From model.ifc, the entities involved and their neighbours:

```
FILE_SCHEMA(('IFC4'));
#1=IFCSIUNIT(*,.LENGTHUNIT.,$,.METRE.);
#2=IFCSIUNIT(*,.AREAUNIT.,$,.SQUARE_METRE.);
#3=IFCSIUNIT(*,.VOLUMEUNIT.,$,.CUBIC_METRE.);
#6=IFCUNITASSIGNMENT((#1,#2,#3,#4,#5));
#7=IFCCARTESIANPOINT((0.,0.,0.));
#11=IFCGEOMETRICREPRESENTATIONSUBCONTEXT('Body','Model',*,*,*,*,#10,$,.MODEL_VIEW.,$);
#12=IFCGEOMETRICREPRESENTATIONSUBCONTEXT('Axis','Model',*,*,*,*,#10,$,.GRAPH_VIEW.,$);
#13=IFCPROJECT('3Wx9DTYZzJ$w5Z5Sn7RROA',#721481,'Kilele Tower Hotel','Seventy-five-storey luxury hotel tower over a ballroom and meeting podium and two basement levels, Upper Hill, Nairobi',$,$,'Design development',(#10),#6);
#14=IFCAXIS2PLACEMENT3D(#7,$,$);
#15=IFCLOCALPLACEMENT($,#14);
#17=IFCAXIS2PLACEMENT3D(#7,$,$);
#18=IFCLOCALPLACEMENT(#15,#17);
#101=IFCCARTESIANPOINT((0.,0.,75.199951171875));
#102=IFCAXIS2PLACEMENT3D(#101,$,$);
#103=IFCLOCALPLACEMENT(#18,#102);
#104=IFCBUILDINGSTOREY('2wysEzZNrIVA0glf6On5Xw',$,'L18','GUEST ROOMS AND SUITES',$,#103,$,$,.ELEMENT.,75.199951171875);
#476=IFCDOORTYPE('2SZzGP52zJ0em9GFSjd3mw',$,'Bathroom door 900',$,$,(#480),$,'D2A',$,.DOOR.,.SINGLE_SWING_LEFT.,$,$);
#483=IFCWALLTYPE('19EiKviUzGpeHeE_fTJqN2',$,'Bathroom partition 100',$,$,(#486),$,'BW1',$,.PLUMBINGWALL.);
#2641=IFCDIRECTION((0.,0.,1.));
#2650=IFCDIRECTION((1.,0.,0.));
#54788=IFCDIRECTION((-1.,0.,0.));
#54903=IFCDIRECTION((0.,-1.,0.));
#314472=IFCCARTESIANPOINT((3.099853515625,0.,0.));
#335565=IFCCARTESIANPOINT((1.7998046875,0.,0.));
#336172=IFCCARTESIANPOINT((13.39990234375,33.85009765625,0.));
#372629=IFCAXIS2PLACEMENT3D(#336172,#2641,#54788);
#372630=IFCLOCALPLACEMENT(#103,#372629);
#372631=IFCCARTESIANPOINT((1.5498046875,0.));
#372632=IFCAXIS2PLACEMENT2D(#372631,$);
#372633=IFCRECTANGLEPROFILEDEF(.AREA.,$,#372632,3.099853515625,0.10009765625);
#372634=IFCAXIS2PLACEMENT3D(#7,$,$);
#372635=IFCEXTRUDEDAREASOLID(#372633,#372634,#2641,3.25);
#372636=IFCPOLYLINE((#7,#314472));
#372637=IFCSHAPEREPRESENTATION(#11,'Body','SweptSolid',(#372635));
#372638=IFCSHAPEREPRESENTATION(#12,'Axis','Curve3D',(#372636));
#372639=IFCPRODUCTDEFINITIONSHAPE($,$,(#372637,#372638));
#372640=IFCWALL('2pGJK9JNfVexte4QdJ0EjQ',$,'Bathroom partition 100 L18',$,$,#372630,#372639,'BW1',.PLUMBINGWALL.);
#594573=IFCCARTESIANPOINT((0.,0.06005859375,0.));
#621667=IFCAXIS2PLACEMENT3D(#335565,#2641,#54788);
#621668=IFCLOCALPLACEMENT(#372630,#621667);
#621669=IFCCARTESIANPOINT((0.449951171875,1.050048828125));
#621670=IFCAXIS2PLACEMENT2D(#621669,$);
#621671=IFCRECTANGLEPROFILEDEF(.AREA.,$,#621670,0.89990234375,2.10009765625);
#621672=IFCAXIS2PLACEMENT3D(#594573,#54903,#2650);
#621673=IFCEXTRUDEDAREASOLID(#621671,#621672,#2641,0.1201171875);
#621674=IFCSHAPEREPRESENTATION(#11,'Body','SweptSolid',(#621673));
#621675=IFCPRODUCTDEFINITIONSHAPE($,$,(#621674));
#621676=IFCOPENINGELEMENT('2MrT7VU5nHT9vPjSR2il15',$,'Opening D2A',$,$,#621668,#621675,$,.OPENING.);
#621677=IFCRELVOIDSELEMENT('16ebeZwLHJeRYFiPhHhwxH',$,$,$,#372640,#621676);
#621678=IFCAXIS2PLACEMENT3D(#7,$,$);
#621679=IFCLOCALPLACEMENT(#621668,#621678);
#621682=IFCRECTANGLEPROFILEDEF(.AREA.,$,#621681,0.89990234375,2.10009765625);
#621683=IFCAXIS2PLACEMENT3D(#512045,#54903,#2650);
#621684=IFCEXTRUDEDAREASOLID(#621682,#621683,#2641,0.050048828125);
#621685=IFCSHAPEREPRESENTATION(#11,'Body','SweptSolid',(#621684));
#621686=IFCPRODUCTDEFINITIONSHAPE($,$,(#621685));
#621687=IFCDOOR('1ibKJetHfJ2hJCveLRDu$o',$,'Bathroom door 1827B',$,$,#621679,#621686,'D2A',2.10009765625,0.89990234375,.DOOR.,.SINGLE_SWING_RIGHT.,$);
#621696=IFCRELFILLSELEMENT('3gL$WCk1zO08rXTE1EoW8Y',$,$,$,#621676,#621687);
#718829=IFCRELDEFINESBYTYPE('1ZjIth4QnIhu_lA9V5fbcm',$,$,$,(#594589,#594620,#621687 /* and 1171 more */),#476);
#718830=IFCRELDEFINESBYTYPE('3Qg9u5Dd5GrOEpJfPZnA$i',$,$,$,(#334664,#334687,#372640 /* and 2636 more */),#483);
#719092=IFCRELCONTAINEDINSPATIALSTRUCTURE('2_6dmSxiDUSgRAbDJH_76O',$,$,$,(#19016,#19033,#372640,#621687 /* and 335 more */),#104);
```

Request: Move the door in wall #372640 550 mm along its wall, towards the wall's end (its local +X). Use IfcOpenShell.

```python
import ifcopenshell
import ifcopenshell.api.geometry
import ifcopenshell.util.placement

model = ifcopenshell.open("model.ifc")

door = model.by_id(621687)
opening = door.FillsVoids[0].RelatingOpeningElement
wall = opening.VoidsElements[0].RelatingBuildingElement

wall_matrix = ifcopenshell.util.placement.get_local_placement(wall.ObjectPlacement)
shift = wall_matrix[:3, 0] * 0.55
before = ifcopenshell.util.placement.get_local_placement(door.ObjectPlacement)[:3, 3].copy()

# The door is placed relative to its opening, so it follows when the opening moves.
matrix = ifcopenshell.util.placement.get_local_placement(opening.ObjectPlacement)
matrix[:3, 3] += shift
ifcopenshell.api.geometry.edit_object_placement(
    model, product=opening, matrix=matrix, is_si=False, should_transform_children=True
)

after = ifcopenshell.util.placement.get_local_placement(door.ObjectPlacement)[:3, 3]
print("door moved by", (after - before).round(3) + 0.0)

model.write("model_edited.ifc")
```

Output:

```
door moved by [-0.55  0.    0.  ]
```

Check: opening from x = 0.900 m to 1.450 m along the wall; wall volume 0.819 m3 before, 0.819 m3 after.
